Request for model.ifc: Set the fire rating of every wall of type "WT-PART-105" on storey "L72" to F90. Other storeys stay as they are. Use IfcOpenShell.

First a look at what the model holds.

```python
import ifcopenshell
import ifcopenshell.util.element

model = ifcopenshell.open("model.ifc")
print(model.schema)
storey = next(s for s in model.by_type("IfcBuildingStorey") if s.Name == "L72")
walls = [e for e in ifcopenshell.util.element.get_decomposition(storey) if e.is_a("IfcWall")]
seen = {}
for e in walls:
    element_type = ifcopenshell.util.element.get_type(e)
    key = (element_type.Name if element_type != e and element_type else None, ifcopenshell.util.element.get_pset(e, "Pset_WallCommon", "FireRating"))
    seen[key] = seen.get(key, 0) + 1
for (name, value), count in sorted(seen.items(), key=str):
    print(count, "x", name, "|", value)
```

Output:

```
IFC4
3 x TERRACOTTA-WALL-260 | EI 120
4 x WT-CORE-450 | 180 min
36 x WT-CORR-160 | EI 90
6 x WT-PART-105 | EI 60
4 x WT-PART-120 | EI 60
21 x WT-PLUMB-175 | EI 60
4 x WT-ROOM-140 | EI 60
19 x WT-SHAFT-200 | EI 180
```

```python
import ifcopenshell
import ifcopenshell.api.pset
import ifcopenshell.util.element

model = ifcopenshell.open("model.ifc")

storey = next(s for s in model.by_type("IfcBuildingStorey") if s.Name == "L72")
walls = [e for e in ifcopenshell.util.element.get_decomposition(storey) if e.is_a("IfcWall")]

count = 0
for e in walls:
    element_type = ifcopenshell.util.element.get_type(e)
    if element_type in (None, e) or element_type.Name != "WT-PART-105":
        continue
    # add_pset returns the element's existing set when there is one.
    pset = ifcopenshell.api.pset.add_pset(model, product=e, name="Pset_WallCommon")
    ifcopenshell.api.pset.edit_pset(model, pset=pset, properties={"FireRating": "F90"})
    count += 1

print(count, "walls updated")

model.write("model_v2.ifc")
```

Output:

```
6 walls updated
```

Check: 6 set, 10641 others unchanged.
